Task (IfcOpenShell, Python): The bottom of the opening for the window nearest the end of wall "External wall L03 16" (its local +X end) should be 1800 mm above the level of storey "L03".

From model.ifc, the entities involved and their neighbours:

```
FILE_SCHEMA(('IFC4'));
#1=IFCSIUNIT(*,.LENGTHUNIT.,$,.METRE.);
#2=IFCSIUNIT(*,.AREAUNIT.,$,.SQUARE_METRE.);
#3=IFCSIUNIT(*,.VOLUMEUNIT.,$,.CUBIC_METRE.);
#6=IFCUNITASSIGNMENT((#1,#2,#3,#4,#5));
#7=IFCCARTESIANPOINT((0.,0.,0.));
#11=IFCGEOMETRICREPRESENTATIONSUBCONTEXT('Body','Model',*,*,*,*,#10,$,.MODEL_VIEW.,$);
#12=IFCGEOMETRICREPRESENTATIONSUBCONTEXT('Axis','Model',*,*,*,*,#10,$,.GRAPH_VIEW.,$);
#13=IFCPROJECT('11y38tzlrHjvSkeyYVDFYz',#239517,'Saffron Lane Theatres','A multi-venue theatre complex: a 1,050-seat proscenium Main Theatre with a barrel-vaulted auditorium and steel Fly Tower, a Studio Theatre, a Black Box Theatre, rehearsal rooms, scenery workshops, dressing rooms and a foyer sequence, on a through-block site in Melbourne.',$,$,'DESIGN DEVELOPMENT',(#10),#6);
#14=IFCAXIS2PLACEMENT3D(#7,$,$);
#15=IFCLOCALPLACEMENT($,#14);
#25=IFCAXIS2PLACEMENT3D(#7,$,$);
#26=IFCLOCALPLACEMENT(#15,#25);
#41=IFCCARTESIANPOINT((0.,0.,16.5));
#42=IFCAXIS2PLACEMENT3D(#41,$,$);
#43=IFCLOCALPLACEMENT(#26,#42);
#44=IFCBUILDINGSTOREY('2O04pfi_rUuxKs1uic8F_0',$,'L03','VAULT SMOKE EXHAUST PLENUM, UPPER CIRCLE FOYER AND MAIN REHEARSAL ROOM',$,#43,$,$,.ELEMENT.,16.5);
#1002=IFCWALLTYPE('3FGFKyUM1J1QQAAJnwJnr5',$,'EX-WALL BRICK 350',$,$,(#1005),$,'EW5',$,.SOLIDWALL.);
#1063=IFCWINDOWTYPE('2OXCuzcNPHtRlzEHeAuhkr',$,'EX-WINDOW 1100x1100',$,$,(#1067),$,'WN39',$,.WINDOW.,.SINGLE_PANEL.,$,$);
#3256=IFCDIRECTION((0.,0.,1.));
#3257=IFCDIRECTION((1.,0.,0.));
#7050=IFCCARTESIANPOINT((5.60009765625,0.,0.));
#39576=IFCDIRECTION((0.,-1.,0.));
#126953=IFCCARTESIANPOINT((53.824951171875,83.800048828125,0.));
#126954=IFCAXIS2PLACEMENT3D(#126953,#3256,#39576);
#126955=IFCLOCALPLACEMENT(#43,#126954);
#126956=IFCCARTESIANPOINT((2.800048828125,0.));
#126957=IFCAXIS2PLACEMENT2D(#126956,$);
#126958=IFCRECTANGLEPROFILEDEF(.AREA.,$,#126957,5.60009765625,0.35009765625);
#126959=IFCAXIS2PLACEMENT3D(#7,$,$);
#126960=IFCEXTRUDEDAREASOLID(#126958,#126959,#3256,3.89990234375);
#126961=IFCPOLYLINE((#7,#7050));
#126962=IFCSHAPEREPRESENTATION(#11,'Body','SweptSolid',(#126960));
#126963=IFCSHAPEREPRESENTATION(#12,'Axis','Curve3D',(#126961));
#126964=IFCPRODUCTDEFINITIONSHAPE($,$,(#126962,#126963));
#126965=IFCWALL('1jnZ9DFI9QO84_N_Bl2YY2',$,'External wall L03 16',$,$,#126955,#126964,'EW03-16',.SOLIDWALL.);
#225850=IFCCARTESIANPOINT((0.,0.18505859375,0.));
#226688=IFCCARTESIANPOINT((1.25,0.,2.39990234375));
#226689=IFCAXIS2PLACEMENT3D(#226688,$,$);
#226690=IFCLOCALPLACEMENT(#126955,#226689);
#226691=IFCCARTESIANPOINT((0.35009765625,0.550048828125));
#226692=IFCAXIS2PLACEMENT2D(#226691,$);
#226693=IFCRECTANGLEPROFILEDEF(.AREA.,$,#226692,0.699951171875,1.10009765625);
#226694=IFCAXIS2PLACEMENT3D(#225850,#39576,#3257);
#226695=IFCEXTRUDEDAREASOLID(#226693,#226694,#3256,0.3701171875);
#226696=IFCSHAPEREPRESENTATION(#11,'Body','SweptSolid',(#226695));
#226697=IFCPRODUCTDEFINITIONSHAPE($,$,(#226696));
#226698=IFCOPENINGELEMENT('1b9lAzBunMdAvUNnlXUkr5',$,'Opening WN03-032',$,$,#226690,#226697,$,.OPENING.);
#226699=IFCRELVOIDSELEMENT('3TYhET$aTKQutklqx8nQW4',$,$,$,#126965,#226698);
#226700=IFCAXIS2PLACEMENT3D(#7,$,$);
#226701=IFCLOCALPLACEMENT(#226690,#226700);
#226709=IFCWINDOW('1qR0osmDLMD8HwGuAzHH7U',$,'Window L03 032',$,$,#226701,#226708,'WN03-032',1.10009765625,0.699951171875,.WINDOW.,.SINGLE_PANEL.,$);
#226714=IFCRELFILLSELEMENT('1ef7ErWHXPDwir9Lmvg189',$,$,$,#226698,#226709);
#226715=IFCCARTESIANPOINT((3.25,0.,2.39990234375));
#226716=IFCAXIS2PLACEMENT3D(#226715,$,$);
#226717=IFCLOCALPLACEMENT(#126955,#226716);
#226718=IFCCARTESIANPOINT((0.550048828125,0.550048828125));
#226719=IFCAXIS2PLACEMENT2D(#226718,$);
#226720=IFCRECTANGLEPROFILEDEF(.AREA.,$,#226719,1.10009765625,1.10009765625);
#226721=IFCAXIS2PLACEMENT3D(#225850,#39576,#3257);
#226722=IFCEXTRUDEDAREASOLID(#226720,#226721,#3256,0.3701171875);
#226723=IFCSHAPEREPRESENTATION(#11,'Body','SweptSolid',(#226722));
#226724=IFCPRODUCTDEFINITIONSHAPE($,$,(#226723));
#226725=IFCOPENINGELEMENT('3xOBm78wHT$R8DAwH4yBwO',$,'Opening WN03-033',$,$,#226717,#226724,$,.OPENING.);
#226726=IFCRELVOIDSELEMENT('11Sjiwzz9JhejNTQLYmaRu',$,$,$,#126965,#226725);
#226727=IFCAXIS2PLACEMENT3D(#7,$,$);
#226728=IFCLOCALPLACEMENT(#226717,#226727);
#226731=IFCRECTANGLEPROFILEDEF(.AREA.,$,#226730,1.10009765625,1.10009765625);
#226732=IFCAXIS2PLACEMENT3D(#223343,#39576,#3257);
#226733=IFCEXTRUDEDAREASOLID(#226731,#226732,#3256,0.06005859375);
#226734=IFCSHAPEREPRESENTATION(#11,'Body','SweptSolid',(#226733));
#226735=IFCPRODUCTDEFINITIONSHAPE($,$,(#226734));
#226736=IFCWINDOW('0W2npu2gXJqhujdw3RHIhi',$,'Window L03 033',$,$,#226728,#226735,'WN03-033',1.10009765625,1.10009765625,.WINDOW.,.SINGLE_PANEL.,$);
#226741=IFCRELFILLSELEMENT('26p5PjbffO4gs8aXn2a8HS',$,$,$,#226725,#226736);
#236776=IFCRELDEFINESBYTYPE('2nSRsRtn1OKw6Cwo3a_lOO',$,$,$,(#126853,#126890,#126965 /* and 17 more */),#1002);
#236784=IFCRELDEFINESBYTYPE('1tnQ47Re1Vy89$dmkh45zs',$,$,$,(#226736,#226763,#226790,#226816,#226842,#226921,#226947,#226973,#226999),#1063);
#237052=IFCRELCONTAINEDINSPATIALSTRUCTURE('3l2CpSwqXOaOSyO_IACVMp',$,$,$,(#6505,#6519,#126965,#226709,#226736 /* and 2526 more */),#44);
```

```python
import numpy as np
import ifcopenshell
import ifcopenshell.api.geometry
import ifcopenshell.geom
import ifcopenshell.util.element
import ifcopenshell.util.placement
import ifcopenshell.util.shape
import ifcopenshell.util.unit

model = ifcopenshell.open("model.ifc")
unit_scale = ifcopenshell.util.unit.calculate_unit_scale(model)

window = model.by_guid("0W2npu2gXJqhujdw3RHIhi")
opening = window.FillsVoids[0].RelatingOpeningElement
storey = ifcopenshell.util.element.get_container(window, ifc_class="IfcBuildingStorey")
level = ifcopenshell.util.placement.get_local_placement(storey.ObjectPlacement)[2, 3]

# The opening's origin need not be at the sill, so measure its lowest point.
shape = ifcopenshell.geom.create_shape(ifcopenshell.geom.settings(), opening)
bottom = ifcopenshell.util.shape.get_shape_bottom_elevation(shape, shape.geometry) / unit_scale
dz = level + 1.8 / unit_scale - bottom

shift = np.array([0.0, 0.0, dz])
# The window is placed relative to its opening, so it follows when the opening moves.
matrix = ifcopenshell.util.placement.get_local_placement(opening.ObjectPlacement)
matrix[:3, 3] += shift
ifcopenshell.api.geometry.edit_object_placement(
    model, product=opening, matrix=matrix, is_si=False, should_transform_children=True
)

print(f"moved by {dz * unit_scale:+.3f} m")

model.write("model_rev.ifc")
```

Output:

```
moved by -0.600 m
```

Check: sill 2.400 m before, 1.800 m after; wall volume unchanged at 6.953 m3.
